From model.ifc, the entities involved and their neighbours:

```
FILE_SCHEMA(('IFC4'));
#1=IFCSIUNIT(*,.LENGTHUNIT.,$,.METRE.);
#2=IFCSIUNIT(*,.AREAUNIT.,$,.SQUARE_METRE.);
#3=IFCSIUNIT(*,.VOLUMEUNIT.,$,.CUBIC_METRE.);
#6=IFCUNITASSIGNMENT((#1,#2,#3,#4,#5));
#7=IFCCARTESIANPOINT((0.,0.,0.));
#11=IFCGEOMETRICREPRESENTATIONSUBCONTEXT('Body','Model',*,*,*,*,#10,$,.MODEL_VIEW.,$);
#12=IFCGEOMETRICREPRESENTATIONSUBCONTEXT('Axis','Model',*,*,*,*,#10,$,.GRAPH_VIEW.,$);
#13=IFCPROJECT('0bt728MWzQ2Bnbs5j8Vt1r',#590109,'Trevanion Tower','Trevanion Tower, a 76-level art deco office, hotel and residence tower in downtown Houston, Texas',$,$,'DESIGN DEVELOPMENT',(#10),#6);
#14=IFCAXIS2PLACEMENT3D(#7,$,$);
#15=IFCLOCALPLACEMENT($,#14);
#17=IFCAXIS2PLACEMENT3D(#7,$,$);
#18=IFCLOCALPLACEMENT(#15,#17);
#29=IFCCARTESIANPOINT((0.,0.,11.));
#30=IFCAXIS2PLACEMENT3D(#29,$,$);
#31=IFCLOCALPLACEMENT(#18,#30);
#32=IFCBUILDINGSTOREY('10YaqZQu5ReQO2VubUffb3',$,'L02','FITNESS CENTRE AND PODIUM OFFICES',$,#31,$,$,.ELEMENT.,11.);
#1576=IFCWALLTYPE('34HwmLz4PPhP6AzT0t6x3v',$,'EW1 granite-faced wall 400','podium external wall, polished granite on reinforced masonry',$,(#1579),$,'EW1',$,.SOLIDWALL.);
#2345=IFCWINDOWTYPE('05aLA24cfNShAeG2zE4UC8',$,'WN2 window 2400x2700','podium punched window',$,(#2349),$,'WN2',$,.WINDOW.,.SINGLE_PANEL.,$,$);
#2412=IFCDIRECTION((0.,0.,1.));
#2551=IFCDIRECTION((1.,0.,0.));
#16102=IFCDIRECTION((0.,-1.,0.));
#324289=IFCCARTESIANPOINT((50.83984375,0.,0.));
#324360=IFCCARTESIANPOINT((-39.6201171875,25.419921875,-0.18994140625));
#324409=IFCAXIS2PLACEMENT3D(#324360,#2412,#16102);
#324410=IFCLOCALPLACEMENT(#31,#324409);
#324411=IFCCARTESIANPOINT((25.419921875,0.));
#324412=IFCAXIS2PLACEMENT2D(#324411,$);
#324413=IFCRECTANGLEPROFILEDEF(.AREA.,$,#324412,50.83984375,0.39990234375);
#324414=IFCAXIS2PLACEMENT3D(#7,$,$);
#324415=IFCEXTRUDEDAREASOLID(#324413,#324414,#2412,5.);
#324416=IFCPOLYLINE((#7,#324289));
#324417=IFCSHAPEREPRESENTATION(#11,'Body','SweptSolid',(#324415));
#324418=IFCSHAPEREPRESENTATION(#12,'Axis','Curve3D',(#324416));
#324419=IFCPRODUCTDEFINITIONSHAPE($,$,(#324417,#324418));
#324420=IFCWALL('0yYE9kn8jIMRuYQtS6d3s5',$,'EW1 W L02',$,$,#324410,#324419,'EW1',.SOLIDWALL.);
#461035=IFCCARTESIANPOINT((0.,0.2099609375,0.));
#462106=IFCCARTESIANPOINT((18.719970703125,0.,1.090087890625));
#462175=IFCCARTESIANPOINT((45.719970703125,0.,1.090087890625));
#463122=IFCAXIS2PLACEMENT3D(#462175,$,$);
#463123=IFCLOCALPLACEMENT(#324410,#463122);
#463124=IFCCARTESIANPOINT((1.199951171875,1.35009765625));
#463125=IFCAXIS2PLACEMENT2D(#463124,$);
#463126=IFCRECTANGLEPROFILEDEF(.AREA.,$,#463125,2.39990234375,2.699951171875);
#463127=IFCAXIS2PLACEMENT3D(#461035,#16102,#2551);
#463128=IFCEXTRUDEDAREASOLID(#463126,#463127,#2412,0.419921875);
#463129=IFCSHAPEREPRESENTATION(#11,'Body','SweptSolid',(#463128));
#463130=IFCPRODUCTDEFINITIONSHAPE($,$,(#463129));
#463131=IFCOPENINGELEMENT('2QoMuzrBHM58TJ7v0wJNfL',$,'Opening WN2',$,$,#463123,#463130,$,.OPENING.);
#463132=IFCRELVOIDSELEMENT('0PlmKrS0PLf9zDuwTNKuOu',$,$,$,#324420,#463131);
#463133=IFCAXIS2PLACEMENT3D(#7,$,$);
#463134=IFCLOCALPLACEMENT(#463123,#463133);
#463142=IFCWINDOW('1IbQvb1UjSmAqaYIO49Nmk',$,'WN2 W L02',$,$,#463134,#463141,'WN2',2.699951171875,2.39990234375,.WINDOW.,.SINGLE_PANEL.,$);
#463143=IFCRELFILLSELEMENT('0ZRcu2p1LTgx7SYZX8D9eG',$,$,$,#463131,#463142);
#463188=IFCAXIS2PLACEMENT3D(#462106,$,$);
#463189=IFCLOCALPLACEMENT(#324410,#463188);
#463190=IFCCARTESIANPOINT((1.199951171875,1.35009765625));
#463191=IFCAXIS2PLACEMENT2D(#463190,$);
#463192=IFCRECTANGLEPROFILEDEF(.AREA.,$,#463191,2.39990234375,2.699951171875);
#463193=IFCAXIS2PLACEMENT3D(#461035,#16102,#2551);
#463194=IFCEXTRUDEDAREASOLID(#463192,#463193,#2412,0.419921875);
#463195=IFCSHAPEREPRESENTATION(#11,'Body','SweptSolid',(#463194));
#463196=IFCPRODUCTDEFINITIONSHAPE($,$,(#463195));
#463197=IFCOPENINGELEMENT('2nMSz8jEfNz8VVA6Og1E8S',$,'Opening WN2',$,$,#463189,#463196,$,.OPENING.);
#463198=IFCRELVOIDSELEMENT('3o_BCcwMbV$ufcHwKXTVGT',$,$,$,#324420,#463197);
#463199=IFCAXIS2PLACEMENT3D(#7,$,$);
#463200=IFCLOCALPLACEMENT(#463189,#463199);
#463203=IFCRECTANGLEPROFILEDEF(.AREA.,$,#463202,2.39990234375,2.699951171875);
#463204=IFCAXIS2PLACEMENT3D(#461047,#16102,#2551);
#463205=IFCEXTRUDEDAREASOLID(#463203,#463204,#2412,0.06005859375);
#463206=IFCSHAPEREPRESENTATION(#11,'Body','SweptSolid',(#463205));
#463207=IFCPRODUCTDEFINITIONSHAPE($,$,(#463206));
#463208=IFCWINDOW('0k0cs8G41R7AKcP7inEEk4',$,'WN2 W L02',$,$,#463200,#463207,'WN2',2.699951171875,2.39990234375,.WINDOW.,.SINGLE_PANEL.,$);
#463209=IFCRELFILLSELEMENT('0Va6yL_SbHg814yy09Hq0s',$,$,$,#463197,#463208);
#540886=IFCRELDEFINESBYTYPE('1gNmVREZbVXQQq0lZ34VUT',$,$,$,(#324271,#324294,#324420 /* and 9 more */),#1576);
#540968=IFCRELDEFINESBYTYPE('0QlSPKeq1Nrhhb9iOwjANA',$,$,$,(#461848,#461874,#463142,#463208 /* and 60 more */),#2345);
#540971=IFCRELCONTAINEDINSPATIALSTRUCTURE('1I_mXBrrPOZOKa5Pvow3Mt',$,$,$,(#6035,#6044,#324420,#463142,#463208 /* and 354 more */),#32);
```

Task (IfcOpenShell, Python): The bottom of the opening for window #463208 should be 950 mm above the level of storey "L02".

```python
import numpy as np
import ifcopenshell
import ifcopenshell.api.geometry
import ifcopenshell.geom
import ifcopenshell.util.element
import ifcopenshell.util.placement
import ifcopenshell.util.shape
import ifcopenshell.util.unit

model = ifcopenshell.open("model.ifc")
unit_scale = ifcopenshell.util.unit.calculate_unit_scale(model)

window = model.by_id(463208)
opening = window.FillsVoids[0].RelatingOpeningElement
storey = ifcopenshell.util.element.get_container(window, ifc_class="IfcBuildingStorey")
level = ifcopenshell.util.placement.get_local_placement(storey.ObjectPlacement)[2, 3]

# The opening's origin need not be at the sill, so measure its lowest point.
shape = ifcopenshell.geom.create_shape(ifcopenshell.geom.settings(), opening)
bottom = ifcopenshell.util.shape.get_shape_bottom_elevation(shape, shape.geometry) / unit_scale
dz = level + 0.95 / unit_scale - bottom

shift = np.array([0.0, 0.0, dz])
# The window is placed relative to its opening, so it follows when the opening moves.
matrix = ifcopenshell.util.placement.get_local_placement(opening.ObjectPlacement)
matrix[:3, 3] += shift
ifcopenshell.api.geometry.edit_object_placement(
    model, product=opening, matrix=matrix, is_si=False, should_transform_children=True
)

print(f"moved by {dz * unit_scale:+.3f} m")

model.write("model_rev.ifc")
```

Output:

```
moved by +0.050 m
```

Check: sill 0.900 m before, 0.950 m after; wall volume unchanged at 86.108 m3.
